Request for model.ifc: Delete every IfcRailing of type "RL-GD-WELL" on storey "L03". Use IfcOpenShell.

First a look at what the model holds.

```python
import ifcopenshell
import ifcopenshell.util.element

model = ifcopenshell.open("model.ifc")
print(model.schema)
storey = next(s for s in model.by_type("IfcBuildingStorey") if s.Name == "L03")
railings = [e for e in ifcopenshell.util.element.get_decomposition(storey) if e.is_a("IfcRailing")]
seen = {}
for e in railings:
    element_type = ifcopenshell.util.element.get_type(e)
    name = element_type.Name if element_type not in (None, e) else None
    seen[name] = seen.get(name, 0) + 1
for name, count in sorted(seen.items(), key=str):
    print(count, "x", name)
```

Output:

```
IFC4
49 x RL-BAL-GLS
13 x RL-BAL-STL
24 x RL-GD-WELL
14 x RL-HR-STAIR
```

```python
import ifcopenshell
import ifcopenshell.api.root
import ifcopenshell.util.element

model = ifcopenshell.open("model.ifc")

storey = next(s for s in model.by_type("IfcBuildingStorey") if s.Name == "L03")
railings = [e for e in ifcopenshell.util.element.get_decomposition(storey) if e.is_a("IfcRailing")]
targets = [e for e in railings if (t := ifcopenshell.util.element.get_type(e)) not in (None, e) and t.Name == "RL-GD-WELL"]

for e in targets:
    ifcopenshell.api.root.remove_product(model, product=e)
print(len(targets), "removed")

model.write("model_v2.ifc")
```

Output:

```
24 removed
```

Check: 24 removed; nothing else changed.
